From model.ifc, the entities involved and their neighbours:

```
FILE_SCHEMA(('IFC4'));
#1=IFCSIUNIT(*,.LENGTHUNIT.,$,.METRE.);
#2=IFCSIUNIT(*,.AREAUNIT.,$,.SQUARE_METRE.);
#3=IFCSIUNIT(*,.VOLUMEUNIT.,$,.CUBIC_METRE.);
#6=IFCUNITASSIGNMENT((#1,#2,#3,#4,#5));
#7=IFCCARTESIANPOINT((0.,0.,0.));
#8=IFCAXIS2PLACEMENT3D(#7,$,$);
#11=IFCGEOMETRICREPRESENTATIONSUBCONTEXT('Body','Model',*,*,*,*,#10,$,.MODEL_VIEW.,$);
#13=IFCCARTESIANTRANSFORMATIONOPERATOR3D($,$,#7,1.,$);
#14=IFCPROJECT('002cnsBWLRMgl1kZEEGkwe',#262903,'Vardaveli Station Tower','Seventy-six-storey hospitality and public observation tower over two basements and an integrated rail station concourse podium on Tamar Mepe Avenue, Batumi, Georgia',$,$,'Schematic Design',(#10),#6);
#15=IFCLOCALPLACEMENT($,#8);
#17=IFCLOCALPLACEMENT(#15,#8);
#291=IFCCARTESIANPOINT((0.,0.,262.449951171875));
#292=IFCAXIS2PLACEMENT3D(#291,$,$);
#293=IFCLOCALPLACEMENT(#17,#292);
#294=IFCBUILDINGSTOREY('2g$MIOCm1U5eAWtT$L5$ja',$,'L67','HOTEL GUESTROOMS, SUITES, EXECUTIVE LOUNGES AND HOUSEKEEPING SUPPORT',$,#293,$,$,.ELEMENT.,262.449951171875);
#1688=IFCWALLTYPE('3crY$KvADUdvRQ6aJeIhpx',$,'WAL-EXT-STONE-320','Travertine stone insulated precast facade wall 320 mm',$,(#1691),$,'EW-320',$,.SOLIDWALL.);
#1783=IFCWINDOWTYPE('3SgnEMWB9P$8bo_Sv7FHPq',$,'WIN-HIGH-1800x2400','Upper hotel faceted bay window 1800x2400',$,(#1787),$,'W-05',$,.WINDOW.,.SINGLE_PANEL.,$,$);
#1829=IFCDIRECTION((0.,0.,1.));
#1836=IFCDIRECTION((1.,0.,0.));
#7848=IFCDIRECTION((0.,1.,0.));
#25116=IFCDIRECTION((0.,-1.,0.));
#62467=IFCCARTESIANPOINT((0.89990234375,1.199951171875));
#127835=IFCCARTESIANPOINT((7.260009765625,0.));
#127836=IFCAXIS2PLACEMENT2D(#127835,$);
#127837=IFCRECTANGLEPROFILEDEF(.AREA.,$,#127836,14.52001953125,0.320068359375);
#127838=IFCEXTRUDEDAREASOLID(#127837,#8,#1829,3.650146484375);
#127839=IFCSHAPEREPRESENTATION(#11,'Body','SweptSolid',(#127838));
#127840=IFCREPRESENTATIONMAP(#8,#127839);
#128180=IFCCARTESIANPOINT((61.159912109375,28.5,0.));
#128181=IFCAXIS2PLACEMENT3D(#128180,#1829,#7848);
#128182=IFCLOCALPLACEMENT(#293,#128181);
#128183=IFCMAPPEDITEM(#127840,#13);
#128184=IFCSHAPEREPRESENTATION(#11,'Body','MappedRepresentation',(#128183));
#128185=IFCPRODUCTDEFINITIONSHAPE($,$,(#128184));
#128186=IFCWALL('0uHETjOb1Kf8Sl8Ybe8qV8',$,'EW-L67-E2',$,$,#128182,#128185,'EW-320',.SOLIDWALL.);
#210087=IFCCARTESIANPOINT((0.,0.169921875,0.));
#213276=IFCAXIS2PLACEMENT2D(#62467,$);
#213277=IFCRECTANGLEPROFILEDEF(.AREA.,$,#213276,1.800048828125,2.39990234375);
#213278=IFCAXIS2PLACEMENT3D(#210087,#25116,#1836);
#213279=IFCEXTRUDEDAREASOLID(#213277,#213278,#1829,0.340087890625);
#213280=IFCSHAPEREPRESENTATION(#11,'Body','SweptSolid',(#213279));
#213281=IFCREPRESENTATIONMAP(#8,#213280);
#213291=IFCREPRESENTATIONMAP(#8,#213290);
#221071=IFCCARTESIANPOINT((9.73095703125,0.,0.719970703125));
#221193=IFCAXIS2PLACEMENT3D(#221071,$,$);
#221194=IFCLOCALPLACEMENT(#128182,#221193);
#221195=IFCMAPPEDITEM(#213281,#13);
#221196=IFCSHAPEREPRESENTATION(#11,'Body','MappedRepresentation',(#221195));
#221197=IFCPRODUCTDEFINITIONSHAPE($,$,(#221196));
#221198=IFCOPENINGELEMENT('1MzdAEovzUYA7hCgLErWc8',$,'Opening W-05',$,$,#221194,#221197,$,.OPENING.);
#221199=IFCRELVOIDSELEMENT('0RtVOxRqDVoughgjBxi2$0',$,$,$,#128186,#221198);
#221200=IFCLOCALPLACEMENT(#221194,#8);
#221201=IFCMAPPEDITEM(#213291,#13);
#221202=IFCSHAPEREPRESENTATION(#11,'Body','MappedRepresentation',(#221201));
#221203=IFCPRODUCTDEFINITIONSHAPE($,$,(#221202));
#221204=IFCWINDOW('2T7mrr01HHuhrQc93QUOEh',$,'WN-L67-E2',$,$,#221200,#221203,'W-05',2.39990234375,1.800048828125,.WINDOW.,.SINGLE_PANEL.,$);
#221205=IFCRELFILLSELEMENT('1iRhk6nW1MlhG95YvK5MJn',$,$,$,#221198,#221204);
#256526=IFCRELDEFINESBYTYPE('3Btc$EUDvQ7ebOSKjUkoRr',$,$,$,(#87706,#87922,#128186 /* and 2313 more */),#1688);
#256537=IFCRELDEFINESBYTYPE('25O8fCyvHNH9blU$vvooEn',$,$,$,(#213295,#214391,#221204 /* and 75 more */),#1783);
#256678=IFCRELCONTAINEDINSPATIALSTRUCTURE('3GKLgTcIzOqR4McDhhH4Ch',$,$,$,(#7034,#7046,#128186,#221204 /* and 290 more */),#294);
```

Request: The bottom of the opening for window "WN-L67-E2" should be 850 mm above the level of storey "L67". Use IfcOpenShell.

```python
import numpy as np
import ifcopenshell
import ifcopenshell.api.geometry
import ifcopenshell.geom
import ifcopenshell.util.element
import ifcopenshell.util.placement
import ifcopenshell.util.shape
import ifcopenshell.util.unit

model = ifcopenshell.open("model.ifc")
unit_scale = ifcopenshell.util.unit.calculate_unit_scale(model)

window = model.by_guid("2T7mrr01HHuhrQc93QUOEh")
opening = window.FillsVoids[0].RelatingOpeningElement
storey = ifcopenshell.util.element.get_container(window, ifc_class="IfcBuildingStorey")
level = ifcopenshell.util.placement.get_local_placement(storey.ObjectPlacement)[2, 3]

# The opening's origin need not be at the sill, so measure its lowest point.
shape = ifcopenshell.geom.create_shape(ifcopenshell.geom.settings(), opening)
bottom = ifcopenshell.util.shape.get_shape_bottom_elevation(shape, shape.geometry) / unit_scale
dz = level + 0.85 - bottom

shift = np.array([0.0, 0.0, dz])
# The window is placed relative to its opening, so it follows when the opening moves.
matrix = ifcopenshell.util.placement.get_local_placement(opening.ObjectPlacement)
matrix[:3, 3] += shift
ifcopenshell.api.geometry.edit_object_placement(
    model, product=opening, matrix=matrix, is_si=False, should_transform_children=True
)

print(f"moved by {dz * unit_scale:+.3f} m")

model.write("model_edited.ifc")
```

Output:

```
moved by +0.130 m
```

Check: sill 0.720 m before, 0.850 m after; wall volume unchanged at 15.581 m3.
